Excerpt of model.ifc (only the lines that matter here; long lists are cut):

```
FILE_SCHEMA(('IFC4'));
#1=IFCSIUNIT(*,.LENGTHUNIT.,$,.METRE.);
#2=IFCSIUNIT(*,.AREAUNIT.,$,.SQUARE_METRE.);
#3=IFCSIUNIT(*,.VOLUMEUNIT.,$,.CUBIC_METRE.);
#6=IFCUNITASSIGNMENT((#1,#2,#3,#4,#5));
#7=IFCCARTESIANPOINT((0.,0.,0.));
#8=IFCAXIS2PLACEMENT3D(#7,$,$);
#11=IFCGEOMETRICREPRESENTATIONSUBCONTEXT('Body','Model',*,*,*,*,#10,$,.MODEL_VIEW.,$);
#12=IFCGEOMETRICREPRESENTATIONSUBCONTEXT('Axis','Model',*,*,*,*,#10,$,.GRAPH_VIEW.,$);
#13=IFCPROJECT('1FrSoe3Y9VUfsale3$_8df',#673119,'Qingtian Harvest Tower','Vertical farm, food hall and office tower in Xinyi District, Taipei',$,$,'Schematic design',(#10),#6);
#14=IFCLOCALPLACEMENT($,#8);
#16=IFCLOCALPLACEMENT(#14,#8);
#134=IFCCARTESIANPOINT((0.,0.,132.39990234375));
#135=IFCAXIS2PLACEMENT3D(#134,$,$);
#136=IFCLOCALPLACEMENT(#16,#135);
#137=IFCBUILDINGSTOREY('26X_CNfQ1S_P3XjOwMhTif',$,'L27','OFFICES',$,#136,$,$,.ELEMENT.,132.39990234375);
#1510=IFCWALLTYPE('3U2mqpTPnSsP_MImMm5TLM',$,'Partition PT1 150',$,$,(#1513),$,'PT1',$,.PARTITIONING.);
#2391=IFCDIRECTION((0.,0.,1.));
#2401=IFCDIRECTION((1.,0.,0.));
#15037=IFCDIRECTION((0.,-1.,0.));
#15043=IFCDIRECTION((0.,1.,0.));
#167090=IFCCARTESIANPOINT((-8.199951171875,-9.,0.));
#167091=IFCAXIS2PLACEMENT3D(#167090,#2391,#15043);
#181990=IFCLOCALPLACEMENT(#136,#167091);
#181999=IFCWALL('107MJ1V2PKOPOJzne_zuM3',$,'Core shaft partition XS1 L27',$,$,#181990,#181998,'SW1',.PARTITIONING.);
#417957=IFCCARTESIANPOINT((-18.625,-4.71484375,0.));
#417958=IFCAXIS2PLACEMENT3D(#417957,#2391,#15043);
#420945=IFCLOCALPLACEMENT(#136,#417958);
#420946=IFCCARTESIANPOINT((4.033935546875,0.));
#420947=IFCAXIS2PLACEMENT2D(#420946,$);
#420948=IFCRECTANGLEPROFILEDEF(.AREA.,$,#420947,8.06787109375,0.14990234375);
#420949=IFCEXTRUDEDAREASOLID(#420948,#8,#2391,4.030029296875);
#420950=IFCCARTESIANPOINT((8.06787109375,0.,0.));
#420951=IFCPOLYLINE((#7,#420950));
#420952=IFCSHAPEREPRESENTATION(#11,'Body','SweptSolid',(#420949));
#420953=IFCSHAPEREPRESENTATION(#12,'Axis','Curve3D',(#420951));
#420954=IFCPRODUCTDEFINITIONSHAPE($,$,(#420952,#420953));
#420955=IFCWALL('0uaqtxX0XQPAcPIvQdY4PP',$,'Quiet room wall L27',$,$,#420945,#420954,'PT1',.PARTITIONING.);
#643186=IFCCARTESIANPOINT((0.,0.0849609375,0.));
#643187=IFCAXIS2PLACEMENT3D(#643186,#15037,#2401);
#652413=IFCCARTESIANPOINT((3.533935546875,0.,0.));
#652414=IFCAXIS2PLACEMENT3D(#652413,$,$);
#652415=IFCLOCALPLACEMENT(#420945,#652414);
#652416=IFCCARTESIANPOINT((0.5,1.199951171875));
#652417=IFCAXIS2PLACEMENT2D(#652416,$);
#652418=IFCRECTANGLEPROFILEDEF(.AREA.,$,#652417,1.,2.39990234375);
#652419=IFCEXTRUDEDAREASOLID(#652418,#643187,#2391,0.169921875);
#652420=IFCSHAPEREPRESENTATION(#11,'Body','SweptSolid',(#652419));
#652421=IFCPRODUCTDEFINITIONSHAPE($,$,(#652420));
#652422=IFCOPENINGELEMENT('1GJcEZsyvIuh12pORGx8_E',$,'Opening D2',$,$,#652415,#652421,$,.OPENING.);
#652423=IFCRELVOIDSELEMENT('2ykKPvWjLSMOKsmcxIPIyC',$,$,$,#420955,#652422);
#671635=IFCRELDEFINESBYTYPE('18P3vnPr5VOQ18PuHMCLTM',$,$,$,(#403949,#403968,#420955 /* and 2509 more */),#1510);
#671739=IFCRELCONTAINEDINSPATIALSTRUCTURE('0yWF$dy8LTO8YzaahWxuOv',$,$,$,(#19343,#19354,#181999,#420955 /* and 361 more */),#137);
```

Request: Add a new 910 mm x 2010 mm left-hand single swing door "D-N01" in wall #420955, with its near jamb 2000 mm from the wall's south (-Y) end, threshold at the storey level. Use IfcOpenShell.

```python
import numpy as np
import ifcopenshell
import ifcopenshell.api.feature
import ifcopenshell.api.geometry
import ifcopenshell.api.root
import ifcopenshell.api.spatial
import ifcopenshell.geom
import ifcopenshell.util.element
import ifcopenshell.util.placement
import ifcopenshell.util.representation
import ifcopenshell.util.shape
import ifcopenshell.util.unit

model = ifcopenshell.open("model.ifc")
unit_scale = ifcopenshell.util.unit.calculate_unit_scale(model)
settings = ifcopenshell.geom.settings()


def volume(element):
    """Net volume in cubic metres, openings subtracted."""
    shape = ifcopenshell.geom.create_shape(settings, element)
    return ifcopenshell.util.shape.get_volume(shape.geometry)


wall = model.by_guid("0uaqtxX0XQPAcPIvQdY4PP")
storey = ifcopenshell.util.element.get_container(wall, ifc_class="IfcBuildingStorey")
context = ifcopenshell.util.representation.get_context(model, "Model", "Body", "MODEL_VIEW")
before = volume(wall)

width, height, from_end, sill = 0.91, 2.01, 2, 0.0  # metres

# The wall runs along its own X axis, and the end named is its -X end.
wall_shape = ifcopenshell.geom.create_shape(settings, wall)
x, y, z = ifcopenshell.util.shape.get_vertices(wall_shape.geometry).T
start = x.min() + from_end
face, thickness = float(y.min()), float(y.max() - y.min())
wall_matrix = ifcopenshell.util.placement.get_local_placement(wall.ObjectPlacement)
level = ifcopenshell.util.placement.get_local_placement(storey.ObjectPlacement)[2, 3]


def in_wall(x, y):
    """Placement at x, y metres in the wall's axes, at sill height."""
    matrix = wall_matrix.copy()
    matrix[:, 3] = wall_matrix @ np.array([x / unit_scale, y / unit_scale, 0.0, 1.0])
    matrix[2, 3] = level + sill / unit_scale
    return matrix


# Opening: a box that overshoots both wall faces by 50 mm.
opening = ifcopenshell.api.root.create_entity(model, ifc_class="IfcOpeningElement", predefined_type="OPENING")
box = ifcopenshell.api.geometry.add_wall_representation(
    model, context=context, length=width, height=height, thickness=thickness + 0.1
)
ifcopenshell.api.geometry.assign_representation(model, product=opening, representation=box)
ifcopenshell.api.geometry.edit_object_placement(model, product=opening, matrix=in_wall(start, face - 0.05), is_si=False)
ifcopenshell.api.feature.add_feature(model, feature=opening, element=wall)

door = ifcopenshell.api.root.create_entity(model, ifc_class="IfcDoor", name="D-N01", predefined_type="DOOR")
door.OverallWidth, door.OverallHeight = width / unit_scale, height / unit_scale
door.OperationType = "SINGLE_SWING_LEFT"
body = ifcopenshell.api.geometry.add_door_representation(
    model,
    context=context,
    overall_width=door.OverallWidth,
    overall_height=door.OverallHeight,
    operation_type="SINGLE_SWING_LEFT",
    lining_properties={"LiningDepth": thickness / unit_scale, "ThresholdDepth": thickness / unit_scale},
)
ifcopenshell.api.geometry.assign_representation(model, product=door, representation=body)
ifcopenshell.api.spatial.assign_container(model, products=[door], relating_structure=storey)
ifcopenshell.api.feature.add_filling(model, opening=opening, element=door)

# The lining spans the wall, so the door starts at the wall face.
ifcopenshell.api.geometry.edit_object_placement(model, product=door, matrix=in_wall(start, face), is_si=False)

after = volume(wall)

print(f"wall volume {before:.3f} -> {after:.3f} m3")

model.write("model_updated.ifc")
```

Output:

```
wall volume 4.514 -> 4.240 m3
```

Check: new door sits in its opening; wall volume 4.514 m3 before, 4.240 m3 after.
